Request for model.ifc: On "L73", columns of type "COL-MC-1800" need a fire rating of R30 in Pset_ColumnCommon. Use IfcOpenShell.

First a look at what the model holds.

```python
import ifcopenshell
import ifcopenshell.util.element

model = ifcopenshell.open("model.ifc")
print(model.schema)
storey = next(s for s in model.by_type("IfcBuildingStorey") if s.Name == "L73")
columns = [e for e in ifcopenshell.util.element.get_decomposition(storey) if e.is_a("IfcColumn")]
seen = {}
for e in columns:
    element_type = ifcopenshell.util.element.get_type(e)
    key = (element_type.Name if element_type != e and element_type else None, ifcopenshell.util.element.get_pset(e, "Pset_ColumnCommon", "FireRating"))
    seen[key] = seen.get(key, 0) + 1
for (name, value), count in sorted(seen.items(), key=str):
    print(count, "x", name, "|", value)
```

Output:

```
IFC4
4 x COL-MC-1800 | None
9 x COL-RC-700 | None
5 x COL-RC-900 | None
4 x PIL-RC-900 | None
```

```python
import ifcopenshell
import ifcopenshell.api.pset
import ifcopenshell.util.element

model = ifcopenshell.open("model.ifc")

storey = next(s for s in model.by_type("IfcBuildingStorey") if s.Name == "L73")
columns = [e for e in ifcopenshell.util.element.get_decomposition(storey) if e.is_a("IfcColumn")]

count = 0
for e in columns:
    element_type = ifcopenshell.util.element.get_type(e)
    if element_type in (None, e) or element_type.Name != "COL-MC-1800":
        continue
    found = ifcopenshell.util.element.get_pset(e, "Pset_ColumnCommon", should_inherit=False)
    if found:
        pset = model.by_id(found["id"])
        if len(ifcopenshell.util.element.get_elements_by_pset(pset)) > 1:
            pset = ifcopenshell.api.pset.unshare_pset(model, products=[e], pset=pset)[0]
    else:
        pset = ifcopenshell.api.pset.add_pset(model, product=e, name="Pset_ColumnCommon")
    ifcopenshell.api.pset.edit_pset(model, pset=pset, properties={"FireRating": "R30"})
    count += 1

print(count, "columns updated")

model.write("model-out.ifc")
```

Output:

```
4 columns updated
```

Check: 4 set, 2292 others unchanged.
